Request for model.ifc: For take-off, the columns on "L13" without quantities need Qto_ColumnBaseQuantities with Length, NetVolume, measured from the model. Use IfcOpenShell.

First a look at what the model holds.

```python
import ifcopenshell
import ifcopenshell.util.element
import ifcopenshell.util.unit

model = ifcopenshell.open("model.ifc")
print(model.schema)
for unit_type in ("LENGTHUNIT", "AREAUNIT", "VOLUMEUNIT"):
    print(unit_type, ifcopenshell.util.unit.calculate_unit_scale(model, unit_type))
storey = next(s for s in model.by_type("IfcBuildingStorey") if s.Name == "L13")
columns = [e for e in ifcopenshell.util.element.get_decomposition(storey) if e.is_a("IfcColumn")]
for e in sorted(columns, key=lambda e: e.id()):
    print(e.id(), e.is_a(), e.Name, list(ifcopenshell.util.element.get_psets(e, qtos_only=True)), sep=" | ")
```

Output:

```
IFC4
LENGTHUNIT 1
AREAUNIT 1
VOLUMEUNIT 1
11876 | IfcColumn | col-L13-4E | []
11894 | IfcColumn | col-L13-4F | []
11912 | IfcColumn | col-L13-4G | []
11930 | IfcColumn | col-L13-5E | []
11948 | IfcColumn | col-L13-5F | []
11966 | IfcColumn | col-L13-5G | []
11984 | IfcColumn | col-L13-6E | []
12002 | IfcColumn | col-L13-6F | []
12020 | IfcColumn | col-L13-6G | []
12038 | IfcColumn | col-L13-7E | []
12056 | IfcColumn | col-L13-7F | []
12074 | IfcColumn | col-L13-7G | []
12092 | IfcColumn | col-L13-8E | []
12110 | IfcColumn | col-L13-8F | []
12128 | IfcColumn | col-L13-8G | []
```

```python
import ifcopenshell
import ifcopenshell.api.pset
import ifcopenshell.geom
import ifcopenshell.util.element
import ifcopenshell.util.shape
import ifcopenshell.util.unit

model = ifcopenshell.open("model.ifc")
unit_scale = ifcopenshell.util.unit.calculate_unit_scale(model)
volume_scale = ifcopenshell.util.unit.calculate_unit_scale(model, "VOLUMEUNIT")
settings = ifcopenshell.geom.settings()

storey = next(s for s in model.by_type("IfcBuildingStorey") if s.Name == "L13")
columns = [e for e in ifcopenshell.util.element.get_decomposition(storey) if e.is_a("IfcColumn")]

for e in sorted(columns, key=lambda e: e.id()):
    if ifcopenshell.util.element.get_psets(e, qtos_only=True, should_inherit=False):
        continue
    # Geometry comes back in metres, in the element's own axes.
    shape = ifcopenshell.geom.create_shape(settings, e)
    values = {
        "Length": ifcopenshell.util.shape.get_z(shape.geometry) / unit_scale,
        "NetVolume": ifcopenshell.util.shape.get_volume(shape.geometry) / volume_scale,
    }
    qto = ifcopenshell.api.pset.add_qto(model, product=e, name="Qto_ColumnBaseQuantities")
    ifcopenshell.api.pset.edit_qto(model, qto=qto, properties=values)
    print(e.id(), {k: round(v, 3) for k, v in values.items()})

model.write("model-out.ifc")
```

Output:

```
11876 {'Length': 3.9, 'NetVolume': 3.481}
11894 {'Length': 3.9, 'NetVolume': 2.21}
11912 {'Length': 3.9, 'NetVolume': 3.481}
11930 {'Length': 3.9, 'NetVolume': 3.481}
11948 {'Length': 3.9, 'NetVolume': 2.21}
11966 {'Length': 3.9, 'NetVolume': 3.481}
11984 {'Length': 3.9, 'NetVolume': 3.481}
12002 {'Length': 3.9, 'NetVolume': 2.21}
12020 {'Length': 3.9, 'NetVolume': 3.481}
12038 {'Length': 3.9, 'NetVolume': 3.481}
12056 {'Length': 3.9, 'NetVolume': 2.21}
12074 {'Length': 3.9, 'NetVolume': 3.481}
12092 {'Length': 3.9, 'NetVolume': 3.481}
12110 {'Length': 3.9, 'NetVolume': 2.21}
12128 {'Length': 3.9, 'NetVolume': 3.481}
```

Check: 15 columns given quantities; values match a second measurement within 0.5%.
